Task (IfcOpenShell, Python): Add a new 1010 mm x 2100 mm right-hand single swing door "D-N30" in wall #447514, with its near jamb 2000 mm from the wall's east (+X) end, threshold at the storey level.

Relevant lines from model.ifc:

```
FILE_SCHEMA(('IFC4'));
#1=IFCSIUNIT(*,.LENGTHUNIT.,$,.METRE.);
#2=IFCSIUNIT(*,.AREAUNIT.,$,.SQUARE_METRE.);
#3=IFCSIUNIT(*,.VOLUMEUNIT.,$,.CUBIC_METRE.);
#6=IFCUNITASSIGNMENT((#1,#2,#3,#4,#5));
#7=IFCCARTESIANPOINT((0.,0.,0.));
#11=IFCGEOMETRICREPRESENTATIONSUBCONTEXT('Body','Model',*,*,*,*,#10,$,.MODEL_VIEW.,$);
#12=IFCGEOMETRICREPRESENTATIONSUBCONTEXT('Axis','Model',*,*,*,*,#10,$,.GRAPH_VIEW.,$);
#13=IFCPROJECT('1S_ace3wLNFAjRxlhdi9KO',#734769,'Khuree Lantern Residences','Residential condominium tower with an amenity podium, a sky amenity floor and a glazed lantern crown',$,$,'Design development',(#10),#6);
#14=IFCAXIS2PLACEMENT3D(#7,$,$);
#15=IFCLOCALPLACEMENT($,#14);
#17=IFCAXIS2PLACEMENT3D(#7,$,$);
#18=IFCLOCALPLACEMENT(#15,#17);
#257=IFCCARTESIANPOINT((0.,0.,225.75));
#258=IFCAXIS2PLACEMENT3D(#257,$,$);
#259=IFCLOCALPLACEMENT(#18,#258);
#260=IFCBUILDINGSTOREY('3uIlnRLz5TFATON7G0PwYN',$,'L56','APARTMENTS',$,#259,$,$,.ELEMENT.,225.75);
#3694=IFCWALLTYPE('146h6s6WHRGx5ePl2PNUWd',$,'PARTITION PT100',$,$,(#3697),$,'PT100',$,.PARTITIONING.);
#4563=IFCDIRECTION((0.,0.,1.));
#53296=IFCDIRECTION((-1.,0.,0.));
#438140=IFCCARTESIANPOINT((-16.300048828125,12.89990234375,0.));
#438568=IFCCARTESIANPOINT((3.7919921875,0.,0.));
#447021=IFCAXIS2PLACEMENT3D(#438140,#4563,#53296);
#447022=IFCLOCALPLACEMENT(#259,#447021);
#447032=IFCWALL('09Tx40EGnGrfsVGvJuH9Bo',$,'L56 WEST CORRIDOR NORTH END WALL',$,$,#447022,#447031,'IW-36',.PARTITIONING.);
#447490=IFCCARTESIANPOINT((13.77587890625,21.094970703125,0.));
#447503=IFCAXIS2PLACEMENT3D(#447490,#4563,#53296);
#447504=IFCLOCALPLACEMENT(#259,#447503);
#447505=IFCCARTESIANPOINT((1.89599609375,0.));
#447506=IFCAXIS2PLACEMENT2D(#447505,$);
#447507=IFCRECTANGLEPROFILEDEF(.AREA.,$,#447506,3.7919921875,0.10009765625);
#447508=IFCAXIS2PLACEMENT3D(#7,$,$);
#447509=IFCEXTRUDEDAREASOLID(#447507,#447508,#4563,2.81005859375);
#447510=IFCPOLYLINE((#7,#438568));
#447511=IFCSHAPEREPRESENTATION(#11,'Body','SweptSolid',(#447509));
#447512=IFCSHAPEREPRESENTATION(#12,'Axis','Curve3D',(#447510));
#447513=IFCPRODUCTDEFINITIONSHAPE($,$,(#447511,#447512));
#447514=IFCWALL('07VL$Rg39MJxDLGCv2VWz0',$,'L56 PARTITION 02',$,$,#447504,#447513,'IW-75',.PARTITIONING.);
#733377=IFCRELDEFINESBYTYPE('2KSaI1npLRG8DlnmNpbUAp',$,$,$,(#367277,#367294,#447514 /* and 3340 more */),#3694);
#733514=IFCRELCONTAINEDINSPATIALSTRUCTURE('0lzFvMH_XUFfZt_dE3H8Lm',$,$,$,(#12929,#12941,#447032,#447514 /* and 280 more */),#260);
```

```python
import numpy as np
import ifcopenshell
import ifcopenshell.api.feature
import ifcopenshell.api.geometry
import ifcopenshell.api.root
import ifcopenshell.api.spatial
import ifcopenshell.geom
import ifcopenshell.util.element
import ifcopenshell.util.placement
import ifcopenshell.util.representation
import ifcopenshell.util.shape
import ifcopenshell.util.unit

model = ifcopenshell.open("model.ifc")
unit_scale = ifcopenshell.util.unit.calculate_unit_scale(model)
settings = ifcopenshell.geom.settings()


def volume(element):
    """Net volume in cubic metres, openings subtracted."""
    shape = ifcopenshell.geom.create_shape(settings, element)
    return ifcopenshell.util.shape.get_volume(shape.geometry)


wall = model.by_id(447514)
storey = ifcopenshell.util.element.get_container(wall, ifc_class="IfcBuildingStorey")
context = ifcopenshell.util.representation.get_context(model, "Model", "Body", "MODEL_VIEW")
before = volume(wall)

width, height, from_end, sill = 1.01, 2.1, 2, 0.0  # metres

# The wall runs along its own X axis, and the end named is its -X end.
wall_shape = ifcopenshell.geom.create_shape(settings, wall)
x, y, z = ifcopenshell.util.shape.get_vertices(wall_shape.geometry).T
start = x.min() + from_end
face, thickness = float(y.min()), float(y.max() - y.min())
wall_matrix = ifcopenshell.util.placement.get_local_placement(wall.ObjectPlacement)
level = ifcopenshell.util.placement.get_local_placement(storey.ObjectPlacement)[2, 3]


def in_wall(x, y):
    """Placement at x, y metres in the wall's axes, at sill height."""
    matrix = wall_matrix.copy()
    matrix[:, 3] = wall_matrix @ np.array([x / unit_scale, y / unit_scale, 0.0, 1.0])
    matrix[2, 3] = level + sill / unit_scale
    return matrix


# Opening: a box that overshoots both wall faces by 50 mm.
opening = ifcopenshell.api.root.create_entity(model, ifc_class="IfcOpeningElement", predefined_type="OPENING")
box = ifcopenshell.api.geometry.add_wall_representation(
    model, context=context, length=width, height=height, thickness=thickness + 0.1
)
ifcopenshell.api.geometry.assign_representation(model, product=opening, representation=box)
ifcopenshell.api.geometry.edit_object_placement(model, product=opening, matrix=in_wall(start, face - 0.05), is_si=False)
ifcopenshell.api.feature.add_feature(model, feature=opening, element=wall)

door = ifcopenshell.api.root.create_entity(model, ifc_class="IfcDoor", name="D-N30", predefined_type="DOOR")
door.OverallWidth, door.OverallHeight = width / unit_scale, height / unit_scale
door.OperationType = "SINGLE_SWING_RIGHT"
body = ifcopenshell.api.geometry.add_door_representation(
    model,
    context=context,
    overall_width=door.OverallWidth,
    overall_height=door.OverallHeight,
    operation_type="SINGLE_SWING_RIGHT",
    lining_properties={"LiningDepth": thickness / unit_scale, "ThresholdDepth": thickness / unit_scale},
)
ifcopenshell.api.geometry.assign_representation(model, product=door, representation=body)
ifcopenshell.api.spatial.assign_container(model, products=[door], relating_structure=storey)
ifcopenshell.api.feature.add_filling(model, opening=opening, element=door)

# The lining spans the wall, so the door starts at the wall face.
ifcopenshell.api.geometry.edit_object_placement(model, product=door, matrix=in_wall(start, face), is_si=False)

after = volume(wall)

print(f"wall volume {before:.3f} -> {after:.3f} m3")

model.write("model_rev.ifc")
```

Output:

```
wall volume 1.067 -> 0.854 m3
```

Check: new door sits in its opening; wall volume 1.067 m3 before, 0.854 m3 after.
